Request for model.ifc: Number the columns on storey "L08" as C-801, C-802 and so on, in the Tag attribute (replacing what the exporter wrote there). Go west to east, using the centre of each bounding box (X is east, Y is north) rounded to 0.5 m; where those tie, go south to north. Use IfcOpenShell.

First a look at what the model holds.

```python
import ifcopenshell
import ifcopenshell.util.element
import ifcopenshell.util.placement

model = ifcopenshell.open("model.ifc")
print(model.schema)
storey = next(s for s in model.by_type("IfcBuildingStorey") if s.Name == "L08")
columns = [e for e in ifcopenshell.util.element.get_decomposition(storey) if e.is_a("IfcColumn")]
for e in sorted(columns, key=lambda e: e.id()):
    origin = ifcopenshell.util.placement.get_local_placement(e.ObjectPlacement)[:3, 3]
    print(e.id(), e.Tag, e.Name, origin.round(2) + 0.0, sep=" | ")
```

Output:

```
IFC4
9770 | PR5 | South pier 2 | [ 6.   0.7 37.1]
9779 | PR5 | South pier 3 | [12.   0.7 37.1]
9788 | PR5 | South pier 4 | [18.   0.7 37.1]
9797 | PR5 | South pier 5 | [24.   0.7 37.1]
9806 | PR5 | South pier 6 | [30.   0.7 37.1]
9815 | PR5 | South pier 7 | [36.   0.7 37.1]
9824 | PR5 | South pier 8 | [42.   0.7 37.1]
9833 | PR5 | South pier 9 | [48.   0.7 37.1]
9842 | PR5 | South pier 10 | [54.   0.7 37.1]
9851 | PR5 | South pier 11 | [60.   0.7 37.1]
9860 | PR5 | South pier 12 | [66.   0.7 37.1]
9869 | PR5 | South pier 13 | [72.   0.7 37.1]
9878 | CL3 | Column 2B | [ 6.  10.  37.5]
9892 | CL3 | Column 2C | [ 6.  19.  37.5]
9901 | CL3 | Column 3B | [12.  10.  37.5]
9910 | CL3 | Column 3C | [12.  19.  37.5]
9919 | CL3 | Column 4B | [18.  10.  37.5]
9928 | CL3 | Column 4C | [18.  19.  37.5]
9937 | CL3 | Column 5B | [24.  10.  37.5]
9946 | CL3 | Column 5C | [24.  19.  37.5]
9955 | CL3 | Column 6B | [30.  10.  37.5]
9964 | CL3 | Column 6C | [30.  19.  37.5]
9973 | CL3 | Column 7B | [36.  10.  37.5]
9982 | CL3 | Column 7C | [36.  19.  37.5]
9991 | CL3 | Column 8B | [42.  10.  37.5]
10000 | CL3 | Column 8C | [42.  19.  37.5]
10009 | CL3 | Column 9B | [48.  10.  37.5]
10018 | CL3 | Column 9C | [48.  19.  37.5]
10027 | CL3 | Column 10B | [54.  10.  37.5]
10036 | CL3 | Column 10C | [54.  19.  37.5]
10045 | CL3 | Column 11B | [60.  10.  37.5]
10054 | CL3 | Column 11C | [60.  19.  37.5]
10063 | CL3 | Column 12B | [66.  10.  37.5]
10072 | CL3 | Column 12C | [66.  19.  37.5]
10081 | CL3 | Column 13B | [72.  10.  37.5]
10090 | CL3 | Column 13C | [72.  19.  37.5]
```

```python
import ifcopenshell
import ifcopenshell.geom
import ifcopenshell.util.element
import ifcopenshell.util.shape

model = ifcopenshell.open("model.ifc")
settings = ifcopenshell.geom.settings()
settings.set("use-world-coords", True)


def centre(element):
    shape = ifcopenshell.geom.create_shape(settings, element)
    return ifcopenshell.util.shape.get_bbox_centroid(shape.geometry)


storey = next(s for s in model.by_type("IfcBuildingStorey") if s.Name == "L08")
columns = [e for e in ifcopenshell.util.element.get_decomposition(storey) if e.is_a("IfcColumn")]

# Insertion points can sit at a corner or the storey origin, so sort by the geometry (in metres).
centres = {e: centre(e) for e in columns}
columns.sort(key=lambda e: (round(centres[e][0] / 0.5), centres[e][1]))

for i, e in enumerate(columns, start=1):
    number = f"C-8{i:02d}"
    e.Tag = number
    print(e.id(), number)

model.write("model_updated.ifc")
```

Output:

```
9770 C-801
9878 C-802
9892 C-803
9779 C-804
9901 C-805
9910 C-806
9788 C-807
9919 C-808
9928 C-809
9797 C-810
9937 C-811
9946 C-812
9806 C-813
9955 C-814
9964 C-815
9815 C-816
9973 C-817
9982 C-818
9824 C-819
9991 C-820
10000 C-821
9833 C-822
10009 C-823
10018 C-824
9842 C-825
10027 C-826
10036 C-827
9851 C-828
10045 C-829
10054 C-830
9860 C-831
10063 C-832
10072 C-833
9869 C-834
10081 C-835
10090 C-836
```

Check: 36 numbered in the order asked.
